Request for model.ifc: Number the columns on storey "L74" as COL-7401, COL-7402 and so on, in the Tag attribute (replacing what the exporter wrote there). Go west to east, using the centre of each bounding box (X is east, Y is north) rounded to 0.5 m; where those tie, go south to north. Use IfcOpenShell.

First a look at what the model holds.

```python
import ifcopenshell
import ifcopenshell.util.element
import ifcopenshell.util.placement

model = ifcopenshell.open("model.ifc")
print(model.schema)
storey = next(s for s in model.by_type("IfcBuildingStorey") if s.Name == "L74")
columns = [e for e in ifcopenshell.util.element.get_decomposition(storey) if e.is_a("IfcColumn")]
for e in sorted(columns, key=lambda e: e.id()):
    origin = ifcopenshell.util.placement.get_local_placement(e.ObjectPlacement)[:3, 3]
    print(e.id(), e.Tag, e.Name, origin.round(2) + 0.0, sep=" | ")
```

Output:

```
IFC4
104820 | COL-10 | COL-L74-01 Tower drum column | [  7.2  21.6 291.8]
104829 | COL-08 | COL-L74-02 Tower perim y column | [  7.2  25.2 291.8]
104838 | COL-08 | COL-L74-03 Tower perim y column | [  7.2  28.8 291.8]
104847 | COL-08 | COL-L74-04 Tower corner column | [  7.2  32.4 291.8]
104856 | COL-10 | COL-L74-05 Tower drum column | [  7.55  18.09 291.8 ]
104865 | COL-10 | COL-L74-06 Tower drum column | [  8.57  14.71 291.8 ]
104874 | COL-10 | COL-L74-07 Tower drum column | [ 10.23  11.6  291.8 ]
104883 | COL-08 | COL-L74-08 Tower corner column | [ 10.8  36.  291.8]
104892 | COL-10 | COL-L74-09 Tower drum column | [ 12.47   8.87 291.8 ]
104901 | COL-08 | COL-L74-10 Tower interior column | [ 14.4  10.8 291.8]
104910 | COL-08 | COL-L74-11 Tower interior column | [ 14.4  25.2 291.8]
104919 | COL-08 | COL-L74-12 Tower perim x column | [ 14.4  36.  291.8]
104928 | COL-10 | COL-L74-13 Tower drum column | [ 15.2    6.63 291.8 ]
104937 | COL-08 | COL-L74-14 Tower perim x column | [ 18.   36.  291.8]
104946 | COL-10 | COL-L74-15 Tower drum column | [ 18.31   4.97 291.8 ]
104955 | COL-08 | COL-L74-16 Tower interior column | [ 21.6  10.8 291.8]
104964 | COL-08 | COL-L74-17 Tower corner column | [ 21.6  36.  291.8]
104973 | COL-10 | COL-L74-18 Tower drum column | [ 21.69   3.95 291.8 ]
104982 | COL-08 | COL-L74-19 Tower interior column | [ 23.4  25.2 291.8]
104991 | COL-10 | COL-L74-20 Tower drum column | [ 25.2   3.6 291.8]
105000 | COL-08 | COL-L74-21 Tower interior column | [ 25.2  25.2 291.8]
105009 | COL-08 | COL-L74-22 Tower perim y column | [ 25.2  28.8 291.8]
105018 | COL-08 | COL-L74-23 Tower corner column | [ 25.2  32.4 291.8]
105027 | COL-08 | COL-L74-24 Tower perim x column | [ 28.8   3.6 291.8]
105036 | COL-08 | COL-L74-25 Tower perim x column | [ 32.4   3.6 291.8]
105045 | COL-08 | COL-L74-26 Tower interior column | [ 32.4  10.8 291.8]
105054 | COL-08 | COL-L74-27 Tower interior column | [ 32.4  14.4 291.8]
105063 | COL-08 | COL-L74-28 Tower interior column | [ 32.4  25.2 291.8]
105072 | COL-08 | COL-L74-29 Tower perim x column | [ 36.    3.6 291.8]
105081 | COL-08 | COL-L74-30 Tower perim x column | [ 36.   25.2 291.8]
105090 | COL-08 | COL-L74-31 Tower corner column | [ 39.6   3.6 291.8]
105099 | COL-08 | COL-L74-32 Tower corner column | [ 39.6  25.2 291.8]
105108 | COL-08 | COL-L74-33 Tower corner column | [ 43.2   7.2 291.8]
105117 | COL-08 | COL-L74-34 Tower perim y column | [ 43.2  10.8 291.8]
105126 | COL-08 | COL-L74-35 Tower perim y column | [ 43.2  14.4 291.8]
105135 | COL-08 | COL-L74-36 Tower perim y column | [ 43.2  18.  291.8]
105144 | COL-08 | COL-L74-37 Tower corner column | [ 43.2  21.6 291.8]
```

```python
import ifcopenshell
import ifcopenshell.geom
import ifcopenshell.util.element
import ifcopenshell.util.shape

model = ifcopenshell.open("model.ifc")
settings = ifcopenshell.geom.settings()
settings.set("use-world-coords", True)


def centre(element):
    shape = ifcopenshell.geom.create_shape(settings, element)
    return ifcopenshell.util.shape.get_bbox_centroid(shape.geometry)


storey = next(s for s in model.by_type("IfcBuildingStorey") if s.Name == "L74")
columns = [e for e in ifcopenshell.util.element.get_decomposition(storey) if e.is_a("IfcColumn")]

# Insertion points can sit at a corner or the storey origin, so sort by the geometry (in metres).
centres = {e: centre(e) for e in columns}
columns.sort(key=lambda e: (round(centres[e][0] / 0.5), centres[e][1]))

for i, e in enumerate(columns, start=1):
    number = f"COL-74{i:02d}"
    e.Tag = number
    print(e.id(), number)

model.write("model-out.ifc")
```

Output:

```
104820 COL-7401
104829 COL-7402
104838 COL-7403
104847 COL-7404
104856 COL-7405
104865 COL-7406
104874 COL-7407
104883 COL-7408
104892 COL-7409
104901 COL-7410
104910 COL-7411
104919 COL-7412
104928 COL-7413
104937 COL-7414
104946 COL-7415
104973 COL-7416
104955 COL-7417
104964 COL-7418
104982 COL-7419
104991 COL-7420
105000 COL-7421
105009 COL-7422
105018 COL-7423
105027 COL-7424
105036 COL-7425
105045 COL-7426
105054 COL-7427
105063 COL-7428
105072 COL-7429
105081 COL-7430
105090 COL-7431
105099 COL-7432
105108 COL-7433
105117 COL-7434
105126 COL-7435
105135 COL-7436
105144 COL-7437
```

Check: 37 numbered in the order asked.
